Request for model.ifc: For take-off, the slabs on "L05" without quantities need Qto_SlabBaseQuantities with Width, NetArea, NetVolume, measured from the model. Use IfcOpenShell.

First a look at what the model holds.

```python
import ifcopenshell
import ifcopenshell.util.element
import ifcopenshell.util.unit

model = ifcopenshell.open("model.ifc")
print(model.schema)
for unit_type in ("LENGTHUNIT", "AREAUNIT", "VOLUMEUNIT"):
    print(unit_type, ifcopenshell.util.unit.calculate_unit_scale(model, unit_type))
storey = next(s for s in model.by_type("IfcBuildingStorey") if s.Name == "L05")
slabs = [e for e in ifcopenshell.util.element.get_decomposition(storey) if e.is_a("IfcSlab")]
for e in sorted(slabs, key=lambda e: e.id()):
    print(e.id(), e.is_a(), e.Name, list(ifcopenshell.util.element.get_psets(e, qtos_only=True)), sep=" | ")
```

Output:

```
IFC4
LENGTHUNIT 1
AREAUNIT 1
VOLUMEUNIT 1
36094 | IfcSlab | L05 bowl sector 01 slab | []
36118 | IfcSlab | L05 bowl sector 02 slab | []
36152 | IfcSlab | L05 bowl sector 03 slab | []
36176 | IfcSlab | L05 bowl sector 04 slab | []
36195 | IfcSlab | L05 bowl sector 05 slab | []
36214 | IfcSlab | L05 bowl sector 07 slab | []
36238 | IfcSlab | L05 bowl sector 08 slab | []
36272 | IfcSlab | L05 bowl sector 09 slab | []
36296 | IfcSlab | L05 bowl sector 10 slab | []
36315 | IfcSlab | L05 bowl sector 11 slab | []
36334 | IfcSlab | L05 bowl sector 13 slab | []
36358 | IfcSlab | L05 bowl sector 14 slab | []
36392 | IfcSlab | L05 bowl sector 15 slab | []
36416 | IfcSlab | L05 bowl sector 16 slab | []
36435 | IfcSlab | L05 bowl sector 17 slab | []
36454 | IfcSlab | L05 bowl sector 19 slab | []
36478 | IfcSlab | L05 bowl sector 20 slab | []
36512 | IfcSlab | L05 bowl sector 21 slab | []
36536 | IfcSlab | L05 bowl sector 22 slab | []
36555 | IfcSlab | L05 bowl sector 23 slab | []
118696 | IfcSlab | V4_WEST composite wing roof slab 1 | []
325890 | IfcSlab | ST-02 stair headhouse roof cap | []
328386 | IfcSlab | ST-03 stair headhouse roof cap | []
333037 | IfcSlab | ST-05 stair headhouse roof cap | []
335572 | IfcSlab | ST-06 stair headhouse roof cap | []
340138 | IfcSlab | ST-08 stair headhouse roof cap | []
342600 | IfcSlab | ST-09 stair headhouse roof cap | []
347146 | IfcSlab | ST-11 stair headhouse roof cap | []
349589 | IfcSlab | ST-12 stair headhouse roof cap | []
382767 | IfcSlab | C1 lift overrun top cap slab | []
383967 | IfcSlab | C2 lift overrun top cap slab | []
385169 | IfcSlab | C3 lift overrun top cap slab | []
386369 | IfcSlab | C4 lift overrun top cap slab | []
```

```python
import ifcopenshell
import ifcopenshell.api.pset
import ifcopenshell.geom
import ifcopenshell.util.element
import ifcopenshell.util.shape
import ifcopenshell.util.unit

model = ifcopenshell.open("model.ifc")
unit_scale = ifcopenshell.util.unit.calculate_unit_scale(model)
area_scale = ifcopenshell.util.unit.calculate_unit_scale(model, "AREAUNIT")
volume_scale = ifcopenshell.util.unit.calculate_unit_scale(model, "VOLUMEUNIT")
settings = ifcopenshell.geom.settings()

storey = next(s for s in model.by_type("IfcBuildingStorey") if s.Name == "L05")
slabs = [e for e in ifcopenshell.util.element.get_decomposition(storey) if e.is_a("IfcSlab")]

for e in sorted(slabs, key=lambda e: e.id()):
    if ifcopenshell.util.element.get_psets(e, qtos_only=True, should_inherit=False):
        continue
    # Geometry comes back in metres, in the element's own axes.
    shape = ifcopenshell.geom.create_shape(settings, e)
    values = {
        "Width": ifcopenshell.util.shape.get_z(shape.geometry) / unit_scale,
        "NetArea": ifcopenshell.util.shape.get_footprint_area(shape.geometry) / area_scale,
        "NetVolume": ifcopenshell.util.shape.get_volume(shape.geometry) / volume_scale,
    }
    qto = ifcopenshell.api.pset.add_qto(model, product=e, name="Qto_SlabBaseQuantities")
    ifcopenshell.api.pset.edit_qto(model, qto=qto, properties=values)
    print(e.id(), {k: round(v, 3) for k, v in values.items()})

model.write("model_v2.ifc")
```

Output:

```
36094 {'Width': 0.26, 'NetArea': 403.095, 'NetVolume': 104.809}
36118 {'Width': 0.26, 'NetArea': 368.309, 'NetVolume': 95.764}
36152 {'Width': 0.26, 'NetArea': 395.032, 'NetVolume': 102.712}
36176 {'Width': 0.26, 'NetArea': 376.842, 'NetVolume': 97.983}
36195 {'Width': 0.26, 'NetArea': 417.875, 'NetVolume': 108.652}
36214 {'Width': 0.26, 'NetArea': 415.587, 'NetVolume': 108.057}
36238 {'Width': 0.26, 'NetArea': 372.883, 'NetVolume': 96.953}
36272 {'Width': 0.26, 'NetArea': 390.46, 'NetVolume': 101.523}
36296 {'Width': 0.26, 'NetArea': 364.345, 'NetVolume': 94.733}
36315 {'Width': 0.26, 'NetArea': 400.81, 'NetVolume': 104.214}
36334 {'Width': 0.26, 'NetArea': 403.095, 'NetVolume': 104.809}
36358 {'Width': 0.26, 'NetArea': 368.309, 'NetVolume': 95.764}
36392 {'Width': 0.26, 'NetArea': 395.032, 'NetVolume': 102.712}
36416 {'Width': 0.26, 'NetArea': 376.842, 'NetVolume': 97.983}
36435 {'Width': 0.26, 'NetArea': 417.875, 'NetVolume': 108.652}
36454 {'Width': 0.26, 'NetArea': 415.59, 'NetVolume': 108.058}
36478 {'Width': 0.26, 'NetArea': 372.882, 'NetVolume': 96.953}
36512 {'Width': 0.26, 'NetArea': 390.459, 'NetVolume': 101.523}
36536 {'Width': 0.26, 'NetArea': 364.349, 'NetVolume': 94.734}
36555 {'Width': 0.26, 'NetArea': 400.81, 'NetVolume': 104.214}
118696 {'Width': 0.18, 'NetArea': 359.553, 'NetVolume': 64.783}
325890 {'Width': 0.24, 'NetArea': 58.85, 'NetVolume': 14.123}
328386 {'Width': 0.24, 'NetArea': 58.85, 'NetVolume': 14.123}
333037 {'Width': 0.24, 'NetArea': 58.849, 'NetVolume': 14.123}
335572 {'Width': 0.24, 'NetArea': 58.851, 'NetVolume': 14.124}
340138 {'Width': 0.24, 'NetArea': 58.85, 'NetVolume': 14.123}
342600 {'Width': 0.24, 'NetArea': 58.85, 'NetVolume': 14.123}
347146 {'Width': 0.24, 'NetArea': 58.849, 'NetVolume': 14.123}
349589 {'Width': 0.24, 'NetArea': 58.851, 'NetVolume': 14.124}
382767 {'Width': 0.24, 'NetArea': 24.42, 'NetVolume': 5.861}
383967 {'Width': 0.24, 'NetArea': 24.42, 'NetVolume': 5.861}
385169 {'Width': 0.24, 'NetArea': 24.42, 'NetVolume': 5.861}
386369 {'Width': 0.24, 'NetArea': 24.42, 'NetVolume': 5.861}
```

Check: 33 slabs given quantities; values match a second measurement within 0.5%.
